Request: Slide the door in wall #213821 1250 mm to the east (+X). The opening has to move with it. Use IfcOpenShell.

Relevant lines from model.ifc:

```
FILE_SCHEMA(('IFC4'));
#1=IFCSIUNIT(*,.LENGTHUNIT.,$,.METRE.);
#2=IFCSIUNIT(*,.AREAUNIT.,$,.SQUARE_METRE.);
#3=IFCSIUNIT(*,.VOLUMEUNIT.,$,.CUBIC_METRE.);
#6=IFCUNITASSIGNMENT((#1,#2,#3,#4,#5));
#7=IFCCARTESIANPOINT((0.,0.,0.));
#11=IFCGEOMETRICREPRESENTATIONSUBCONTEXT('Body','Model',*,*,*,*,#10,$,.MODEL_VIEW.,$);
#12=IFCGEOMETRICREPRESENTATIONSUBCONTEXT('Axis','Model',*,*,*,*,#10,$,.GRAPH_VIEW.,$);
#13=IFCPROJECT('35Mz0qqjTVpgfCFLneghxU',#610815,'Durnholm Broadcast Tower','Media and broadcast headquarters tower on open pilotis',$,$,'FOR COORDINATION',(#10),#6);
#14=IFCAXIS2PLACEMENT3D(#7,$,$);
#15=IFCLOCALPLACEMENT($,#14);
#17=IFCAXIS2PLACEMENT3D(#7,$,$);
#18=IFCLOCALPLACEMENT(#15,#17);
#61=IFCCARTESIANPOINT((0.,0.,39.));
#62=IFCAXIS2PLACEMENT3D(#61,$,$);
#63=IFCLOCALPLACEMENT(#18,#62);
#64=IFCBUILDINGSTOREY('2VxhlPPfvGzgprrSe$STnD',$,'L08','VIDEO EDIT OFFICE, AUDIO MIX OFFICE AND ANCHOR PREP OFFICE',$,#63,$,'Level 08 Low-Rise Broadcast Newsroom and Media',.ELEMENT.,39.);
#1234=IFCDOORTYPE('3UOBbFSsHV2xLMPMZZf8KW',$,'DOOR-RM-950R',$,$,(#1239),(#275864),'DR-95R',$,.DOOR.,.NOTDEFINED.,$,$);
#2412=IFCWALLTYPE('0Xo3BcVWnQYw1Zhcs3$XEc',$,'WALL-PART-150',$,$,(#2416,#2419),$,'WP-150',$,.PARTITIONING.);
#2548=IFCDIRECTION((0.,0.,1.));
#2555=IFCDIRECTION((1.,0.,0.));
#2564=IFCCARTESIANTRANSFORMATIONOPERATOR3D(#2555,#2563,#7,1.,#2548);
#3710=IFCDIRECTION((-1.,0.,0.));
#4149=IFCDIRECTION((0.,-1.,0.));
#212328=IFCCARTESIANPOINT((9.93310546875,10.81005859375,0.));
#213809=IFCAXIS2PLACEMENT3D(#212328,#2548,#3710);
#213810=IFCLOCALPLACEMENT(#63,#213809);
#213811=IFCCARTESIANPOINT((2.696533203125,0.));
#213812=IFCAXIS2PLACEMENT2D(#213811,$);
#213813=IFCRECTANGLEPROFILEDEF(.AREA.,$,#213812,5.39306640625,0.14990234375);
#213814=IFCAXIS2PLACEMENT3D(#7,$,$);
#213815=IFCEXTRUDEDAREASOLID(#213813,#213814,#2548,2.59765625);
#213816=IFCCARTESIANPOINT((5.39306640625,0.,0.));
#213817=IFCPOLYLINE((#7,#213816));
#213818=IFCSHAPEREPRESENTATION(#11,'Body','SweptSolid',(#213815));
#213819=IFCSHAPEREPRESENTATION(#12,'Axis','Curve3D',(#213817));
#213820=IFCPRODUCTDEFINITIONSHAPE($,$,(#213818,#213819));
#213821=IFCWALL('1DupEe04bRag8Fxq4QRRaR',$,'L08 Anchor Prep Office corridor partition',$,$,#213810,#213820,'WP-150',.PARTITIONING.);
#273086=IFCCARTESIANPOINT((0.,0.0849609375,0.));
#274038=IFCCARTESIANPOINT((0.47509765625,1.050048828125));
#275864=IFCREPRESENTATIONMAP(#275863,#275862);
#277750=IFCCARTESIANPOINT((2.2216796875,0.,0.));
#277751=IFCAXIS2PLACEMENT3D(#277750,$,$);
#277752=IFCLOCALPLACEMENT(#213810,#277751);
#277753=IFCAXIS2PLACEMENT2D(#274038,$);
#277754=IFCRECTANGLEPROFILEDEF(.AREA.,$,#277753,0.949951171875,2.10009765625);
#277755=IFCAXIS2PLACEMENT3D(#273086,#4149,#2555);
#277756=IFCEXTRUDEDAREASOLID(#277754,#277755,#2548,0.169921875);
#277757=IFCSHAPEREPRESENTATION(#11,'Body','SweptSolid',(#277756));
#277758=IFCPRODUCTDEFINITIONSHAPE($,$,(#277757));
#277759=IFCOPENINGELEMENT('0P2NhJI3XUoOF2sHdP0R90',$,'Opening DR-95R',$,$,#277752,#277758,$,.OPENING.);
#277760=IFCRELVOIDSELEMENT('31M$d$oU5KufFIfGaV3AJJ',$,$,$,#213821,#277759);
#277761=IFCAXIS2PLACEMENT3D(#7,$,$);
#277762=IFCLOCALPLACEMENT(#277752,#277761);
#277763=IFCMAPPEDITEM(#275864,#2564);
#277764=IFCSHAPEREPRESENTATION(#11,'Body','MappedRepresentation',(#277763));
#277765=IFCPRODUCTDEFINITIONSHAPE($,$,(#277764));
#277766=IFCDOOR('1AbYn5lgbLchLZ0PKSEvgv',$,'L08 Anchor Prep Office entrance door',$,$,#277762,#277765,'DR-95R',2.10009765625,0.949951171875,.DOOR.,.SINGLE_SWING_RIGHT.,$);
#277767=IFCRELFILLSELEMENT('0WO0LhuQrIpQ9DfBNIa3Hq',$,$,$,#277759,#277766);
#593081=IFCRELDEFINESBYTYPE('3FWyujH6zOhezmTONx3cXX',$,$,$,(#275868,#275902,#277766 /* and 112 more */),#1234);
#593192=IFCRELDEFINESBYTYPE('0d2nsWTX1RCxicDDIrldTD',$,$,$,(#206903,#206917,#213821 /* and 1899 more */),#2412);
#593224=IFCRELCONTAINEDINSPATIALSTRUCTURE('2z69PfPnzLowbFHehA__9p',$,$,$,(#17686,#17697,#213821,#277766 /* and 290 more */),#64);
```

```python
import ifcopenshell
import ifcopenshell.api.geometry
import ifcopenshell.util.placement
import ifcopenshell.util.unit

model = ifcopenshell.open("model.ifc")
unit_scale = ifcopenshell.util.unit.calculate_unit_scale(model)

door = model.by_guid("1AbYn5lgbLchLZ0PKSEvgv")
opening = door.FillsVoids[0].RelatingOpeningElement
wall = opening.VoidsElements[0].RelatingBuildingElement

wall_matrix = ifcopenshell.util.placement.get_local_placement(wall.ObjectPlacement)
shift = wall_matrix[:3, 0] * -1.25 / unit_scale
before = ifcopenshell.util.placement.get_local_placement(door.ObjectPlacement)[:3, 3].copy()

# The door is placed relative to its opening, so it follows when the opening moves.
matrix = ifcopenshell.util.placement.get_local_placement(opening.ObjectPlacement)
matrix[:3, 3] += shift
ifcopenshell.api.geometry.edit_object_placement(
    model, product=opening, matrix=matrix, is_si=False, should_transform_children=True
)

after = ifcopenshell.util.placement.get_local_placement(door.ObjectPlacement)[:3, 3]
print("door moved by", (after - before).round(3) + 0.0)

model.write("model_updated.ifc")
```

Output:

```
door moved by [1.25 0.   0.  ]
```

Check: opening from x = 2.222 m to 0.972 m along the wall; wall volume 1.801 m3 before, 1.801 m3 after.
